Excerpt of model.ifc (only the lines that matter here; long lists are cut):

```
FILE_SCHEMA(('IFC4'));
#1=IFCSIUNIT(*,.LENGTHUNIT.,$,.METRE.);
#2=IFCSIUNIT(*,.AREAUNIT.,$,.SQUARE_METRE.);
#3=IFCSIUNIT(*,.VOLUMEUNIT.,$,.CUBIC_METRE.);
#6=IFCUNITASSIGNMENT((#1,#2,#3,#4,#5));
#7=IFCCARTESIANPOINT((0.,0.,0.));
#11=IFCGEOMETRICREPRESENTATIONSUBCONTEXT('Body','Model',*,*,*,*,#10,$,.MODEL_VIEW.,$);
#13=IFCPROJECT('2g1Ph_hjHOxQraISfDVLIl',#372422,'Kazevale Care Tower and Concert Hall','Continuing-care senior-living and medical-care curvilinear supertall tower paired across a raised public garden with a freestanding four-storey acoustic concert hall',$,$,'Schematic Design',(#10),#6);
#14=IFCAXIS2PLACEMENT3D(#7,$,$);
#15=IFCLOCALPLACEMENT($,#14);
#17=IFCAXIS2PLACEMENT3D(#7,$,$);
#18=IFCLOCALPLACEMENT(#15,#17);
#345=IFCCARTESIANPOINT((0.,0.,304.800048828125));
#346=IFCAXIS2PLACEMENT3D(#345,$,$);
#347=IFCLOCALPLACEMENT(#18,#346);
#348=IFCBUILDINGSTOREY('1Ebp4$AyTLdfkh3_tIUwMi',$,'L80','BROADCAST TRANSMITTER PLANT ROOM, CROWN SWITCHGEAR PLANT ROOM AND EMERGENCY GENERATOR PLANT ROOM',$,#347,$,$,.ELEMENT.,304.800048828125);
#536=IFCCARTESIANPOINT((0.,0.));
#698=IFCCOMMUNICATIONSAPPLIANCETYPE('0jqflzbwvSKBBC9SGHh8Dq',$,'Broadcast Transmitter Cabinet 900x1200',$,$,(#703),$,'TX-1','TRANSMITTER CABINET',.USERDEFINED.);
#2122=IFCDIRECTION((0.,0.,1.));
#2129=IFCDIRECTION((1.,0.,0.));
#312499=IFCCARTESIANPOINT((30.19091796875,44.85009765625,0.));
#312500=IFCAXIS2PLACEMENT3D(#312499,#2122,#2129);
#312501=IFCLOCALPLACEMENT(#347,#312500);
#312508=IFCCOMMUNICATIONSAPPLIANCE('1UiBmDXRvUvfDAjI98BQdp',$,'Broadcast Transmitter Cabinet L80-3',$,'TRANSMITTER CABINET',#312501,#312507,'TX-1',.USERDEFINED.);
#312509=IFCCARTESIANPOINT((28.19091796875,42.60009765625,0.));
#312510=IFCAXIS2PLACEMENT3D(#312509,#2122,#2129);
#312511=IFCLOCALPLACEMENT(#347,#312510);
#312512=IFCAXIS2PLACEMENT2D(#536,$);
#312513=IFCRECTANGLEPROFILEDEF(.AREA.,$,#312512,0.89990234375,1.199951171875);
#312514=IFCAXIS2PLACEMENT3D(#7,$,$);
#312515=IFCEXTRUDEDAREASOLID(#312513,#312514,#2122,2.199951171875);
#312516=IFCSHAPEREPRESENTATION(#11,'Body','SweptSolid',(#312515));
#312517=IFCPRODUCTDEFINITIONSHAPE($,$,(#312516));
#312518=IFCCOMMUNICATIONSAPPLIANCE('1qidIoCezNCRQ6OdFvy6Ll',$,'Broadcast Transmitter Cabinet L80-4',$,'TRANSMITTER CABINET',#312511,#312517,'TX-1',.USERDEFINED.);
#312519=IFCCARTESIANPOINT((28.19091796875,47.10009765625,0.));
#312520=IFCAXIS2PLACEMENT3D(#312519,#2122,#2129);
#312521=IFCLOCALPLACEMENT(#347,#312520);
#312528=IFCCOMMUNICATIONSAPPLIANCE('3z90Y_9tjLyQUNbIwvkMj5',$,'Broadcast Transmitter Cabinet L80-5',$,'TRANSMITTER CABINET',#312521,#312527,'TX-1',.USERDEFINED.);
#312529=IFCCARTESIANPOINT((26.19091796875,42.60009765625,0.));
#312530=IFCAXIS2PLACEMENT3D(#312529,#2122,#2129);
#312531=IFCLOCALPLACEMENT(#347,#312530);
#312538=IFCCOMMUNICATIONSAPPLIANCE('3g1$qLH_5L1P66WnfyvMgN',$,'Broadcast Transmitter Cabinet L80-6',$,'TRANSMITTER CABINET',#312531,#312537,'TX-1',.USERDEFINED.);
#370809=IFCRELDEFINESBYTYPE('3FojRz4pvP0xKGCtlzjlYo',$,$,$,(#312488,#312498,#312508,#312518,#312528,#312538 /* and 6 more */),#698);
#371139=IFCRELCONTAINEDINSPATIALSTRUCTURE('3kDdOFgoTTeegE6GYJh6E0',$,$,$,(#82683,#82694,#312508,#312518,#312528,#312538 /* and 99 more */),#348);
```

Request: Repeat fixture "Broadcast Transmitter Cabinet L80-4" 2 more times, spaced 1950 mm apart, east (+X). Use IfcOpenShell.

```python
import numpy as np
import ifcopenshell
import ifcopenshell.api.geometry
import ifcopenshell.api.root
import ifcopenshell.util.element
import ifcopenshell.util.placement

model = ifcopenshell.open("model.ifc")

source = model.by_guid("1qidIoCezNCRQ6OdFvy6Ll")
base = ifcopenshell.util.placement.get_local_placement(source.ObjectPlacement)
step = np.array([1.0, 0.0, 0.0]) * 1.95

for i in range(1, 3):
    copy = ifcopenshell.api.root.copy_class(model, product=source)
    copy.Representation = ifcopenshell.util.element.copy_deep(
        model, source.Representation, exclude=["IfcGeometricRepresentationContext", "IfcRepresentationMap"]
    )
    copy.Tag = None
    matrix = base.copy()
    matrix[:3, 3] += i * step
    print("added at", matrix[:3, 3].round(3) + 0.0)
    ifcopenshell.api.geometry.edit_object_placement(model, product=copy, matrix=matrix, is_si=False)

model.write("model_updated.ifc")
```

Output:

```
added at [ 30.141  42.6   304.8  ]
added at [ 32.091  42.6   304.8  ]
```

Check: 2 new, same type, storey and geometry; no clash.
